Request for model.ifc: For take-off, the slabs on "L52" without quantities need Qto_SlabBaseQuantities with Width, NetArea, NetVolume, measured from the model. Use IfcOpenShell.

First a look at what the model holds.

```python
import ifcopenshell
import ifcopenshell.util.element
import ifcopenshell.util.unit

model = ifcopenshell.open("model.ifc")
print(model.schema)
for unit_type in ("LENGTHUNIT", "AREAUNIT", "VOLUMEUNIT"):
    print(unit_type, ifcopenshell.util.unit.calculate_unit_scale(model, unit_type))
storey = next(s for s in model.by_type("IfcBuildingStorey") if s.Name == "L52")
slabs = [e for e in ifcopenshell.util.element.get_decomposition(storey) if e.is_a("IfcSlab")]
for e in sorted(slabs, key=lambda e: e.id()):
    print(e.id(), e.is_a(), e.Name, list(ifcopenshell.util.element.get_psets(e, qtos_only=True)), sep=" | ")
```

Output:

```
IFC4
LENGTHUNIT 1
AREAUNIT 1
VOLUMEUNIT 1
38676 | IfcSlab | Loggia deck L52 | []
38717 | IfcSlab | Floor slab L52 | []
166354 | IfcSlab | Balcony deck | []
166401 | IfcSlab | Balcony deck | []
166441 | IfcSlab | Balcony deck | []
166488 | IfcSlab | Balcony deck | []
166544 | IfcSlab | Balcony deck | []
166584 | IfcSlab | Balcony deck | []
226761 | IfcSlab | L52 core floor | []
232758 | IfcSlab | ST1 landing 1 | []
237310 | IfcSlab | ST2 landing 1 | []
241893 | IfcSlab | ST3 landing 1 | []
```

```python
import ifcopenshell
import ifcopenshell.api.pset
import ifcopenshell.geom
import ifcopenshell.util.element
import ifcopenshell.util.shape
import ifcopenshell.util.unit

model = ifcopenshell.open("model.ifc")
unit_scale = ifcopenshell.util.unit.calculate_unit_scale(model)
area_scale = ifcopenshell.util.unit.calculate_unit_scale(model, "AREAUNIT")
volume_scale = ifcopenshell.util.unit.calculate_unit_scale(model, "VOLUMEUNIT")
settings = ifcopenshell.geom.settings()

storey = next(s for s in model.by_type("IfcBuildingStorey") if s.Name == "L52")
slabs = [e for e in ifcopenshell.util.element.get_decomposition(storey) if e.is_a("IfcSlab")]

for e in sorted(slabs, key=lambda e: e.id()):
    if ifcopenshell.util.element.get_psets(e, qtos_only=True, should_inherit=False):
        continue
    # Geometry comes back in metres, in the element's own axes.
    shape = ifcopenshell.geom.create_shape(settings, e)
    values = {
        "Width": ifcopenshell.util.shape.get_z(shape.geometry) / unit_scale,
        "NetArea": ifcopenshell.util.shape.get_footprint_area(shape.geometry) / area_scale,
        "NetVolume": ifcopenshell.util.shape.get_volume(shape.geometry) / volume_scale,
    }
    qto = ifcopenshell.api.pset.add_qto(model, product=e, name="Qto_SlabBaseQuantities")
    ifcopenshell.api.pset.edit_qto(model, qto=qto, properties=values)
    print(e.id(), {k: round(v, 3) for k, v in values.items()})

model.write("model_edited.ifc")
```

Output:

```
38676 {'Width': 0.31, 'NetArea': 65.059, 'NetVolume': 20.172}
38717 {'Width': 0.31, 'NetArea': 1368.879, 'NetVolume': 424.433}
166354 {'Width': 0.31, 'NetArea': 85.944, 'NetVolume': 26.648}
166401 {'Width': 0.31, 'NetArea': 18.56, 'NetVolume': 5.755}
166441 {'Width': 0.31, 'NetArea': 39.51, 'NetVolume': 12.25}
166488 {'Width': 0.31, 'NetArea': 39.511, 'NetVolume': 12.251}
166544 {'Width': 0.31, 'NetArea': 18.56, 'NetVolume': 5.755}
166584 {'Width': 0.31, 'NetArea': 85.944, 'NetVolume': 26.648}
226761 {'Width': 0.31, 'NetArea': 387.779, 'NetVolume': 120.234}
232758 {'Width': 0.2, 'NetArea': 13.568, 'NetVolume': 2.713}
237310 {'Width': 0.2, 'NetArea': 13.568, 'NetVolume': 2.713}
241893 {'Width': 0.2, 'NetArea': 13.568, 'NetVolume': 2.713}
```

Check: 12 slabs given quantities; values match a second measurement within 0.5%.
